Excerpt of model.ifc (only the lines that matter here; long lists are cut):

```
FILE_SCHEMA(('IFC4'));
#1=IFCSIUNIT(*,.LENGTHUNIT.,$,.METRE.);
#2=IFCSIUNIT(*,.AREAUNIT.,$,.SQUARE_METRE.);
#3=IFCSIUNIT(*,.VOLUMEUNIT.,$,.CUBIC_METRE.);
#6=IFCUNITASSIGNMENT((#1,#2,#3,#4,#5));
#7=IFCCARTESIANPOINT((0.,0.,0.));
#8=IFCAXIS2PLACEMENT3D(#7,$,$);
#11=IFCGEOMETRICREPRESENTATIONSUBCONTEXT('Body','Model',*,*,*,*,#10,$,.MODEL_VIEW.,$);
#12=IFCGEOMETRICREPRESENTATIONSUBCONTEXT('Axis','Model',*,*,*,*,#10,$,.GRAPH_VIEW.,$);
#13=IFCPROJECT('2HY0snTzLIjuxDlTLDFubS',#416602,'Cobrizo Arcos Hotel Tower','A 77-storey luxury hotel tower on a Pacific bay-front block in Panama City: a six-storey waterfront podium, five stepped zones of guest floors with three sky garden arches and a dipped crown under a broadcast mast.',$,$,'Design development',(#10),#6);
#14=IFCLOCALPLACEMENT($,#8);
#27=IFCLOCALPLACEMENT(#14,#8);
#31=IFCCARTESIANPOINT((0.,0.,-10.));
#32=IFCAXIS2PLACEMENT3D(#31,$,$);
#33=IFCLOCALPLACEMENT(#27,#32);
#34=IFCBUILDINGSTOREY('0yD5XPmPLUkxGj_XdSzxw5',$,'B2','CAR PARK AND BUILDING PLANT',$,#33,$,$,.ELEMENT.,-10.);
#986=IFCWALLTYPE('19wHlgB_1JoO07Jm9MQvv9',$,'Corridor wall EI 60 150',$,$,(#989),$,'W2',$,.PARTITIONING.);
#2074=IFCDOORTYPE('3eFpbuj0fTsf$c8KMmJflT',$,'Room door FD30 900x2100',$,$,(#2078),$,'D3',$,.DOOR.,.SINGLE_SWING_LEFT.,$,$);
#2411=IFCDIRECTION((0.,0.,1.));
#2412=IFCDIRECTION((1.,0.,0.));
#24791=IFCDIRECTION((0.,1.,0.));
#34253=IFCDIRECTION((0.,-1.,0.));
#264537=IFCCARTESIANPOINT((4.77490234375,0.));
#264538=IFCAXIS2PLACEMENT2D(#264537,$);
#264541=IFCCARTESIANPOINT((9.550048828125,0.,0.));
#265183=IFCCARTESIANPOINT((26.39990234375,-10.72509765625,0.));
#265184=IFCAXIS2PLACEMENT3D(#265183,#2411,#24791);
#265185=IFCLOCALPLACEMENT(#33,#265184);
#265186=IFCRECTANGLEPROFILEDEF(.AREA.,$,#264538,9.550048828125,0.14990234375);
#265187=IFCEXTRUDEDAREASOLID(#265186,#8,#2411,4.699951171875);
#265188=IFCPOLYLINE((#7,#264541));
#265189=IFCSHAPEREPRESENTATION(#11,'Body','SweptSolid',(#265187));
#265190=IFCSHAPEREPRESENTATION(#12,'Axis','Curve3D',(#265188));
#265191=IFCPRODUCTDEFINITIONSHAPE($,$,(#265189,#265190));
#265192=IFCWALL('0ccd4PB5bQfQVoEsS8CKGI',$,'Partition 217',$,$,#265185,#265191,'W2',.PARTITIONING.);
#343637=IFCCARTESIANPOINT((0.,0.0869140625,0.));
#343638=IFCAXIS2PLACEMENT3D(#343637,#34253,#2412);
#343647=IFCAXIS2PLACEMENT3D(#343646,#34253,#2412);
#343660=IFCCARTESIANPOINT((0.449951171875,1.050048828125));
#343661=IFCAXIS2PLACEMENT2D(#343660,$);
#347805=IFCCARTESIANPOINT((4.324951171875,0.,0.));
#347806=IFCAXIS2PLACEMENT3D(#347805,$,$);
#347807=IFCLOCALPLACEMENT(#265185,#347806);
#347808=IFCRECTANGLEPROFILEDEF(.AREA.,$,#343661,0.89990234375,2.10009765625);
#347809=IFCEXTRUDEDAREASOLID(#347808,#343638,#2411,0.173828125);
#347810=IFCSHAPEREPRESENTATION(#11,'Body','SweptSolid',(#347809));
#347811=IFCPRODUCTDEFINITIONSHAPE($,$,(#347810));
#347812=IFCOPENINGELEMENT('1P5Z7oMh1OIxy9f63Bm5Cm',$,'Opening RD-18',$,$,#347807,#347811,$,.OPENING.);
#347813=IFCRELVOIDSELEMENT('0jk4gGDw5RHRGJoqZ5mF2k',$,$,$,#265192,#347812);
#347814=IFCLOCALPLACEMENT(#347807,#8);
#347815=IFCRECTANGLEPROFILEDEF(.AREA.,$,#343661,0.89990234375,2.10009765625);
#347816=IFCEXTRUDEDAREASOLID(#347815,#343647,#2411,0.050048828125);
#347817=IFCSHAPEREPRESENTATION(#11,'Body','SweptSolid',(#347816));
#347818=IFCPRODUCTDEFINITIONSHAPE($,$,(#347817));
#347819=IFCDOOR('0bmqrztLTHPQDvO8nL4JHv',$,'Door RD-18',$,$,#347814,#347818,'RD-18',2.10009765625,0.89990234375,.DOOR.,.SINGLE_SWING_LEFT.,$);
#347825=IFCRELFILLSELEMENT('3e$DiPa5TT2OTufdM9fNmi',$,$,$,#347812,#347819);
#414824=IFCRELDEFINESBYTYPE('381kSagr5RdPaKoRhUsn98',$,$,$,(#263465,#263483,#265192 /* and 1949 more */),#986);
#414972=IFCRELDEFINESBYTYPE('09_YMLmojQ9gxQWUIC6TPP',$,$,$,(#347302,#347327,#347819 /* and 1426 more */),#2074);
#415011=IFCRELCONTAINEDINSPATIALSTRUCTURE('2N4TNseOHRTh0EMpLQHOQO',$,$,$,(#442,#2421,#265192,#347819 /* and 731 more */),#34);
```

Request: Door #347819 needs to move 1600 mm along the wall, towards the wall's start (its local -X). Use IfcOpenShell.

```python
import ifcopenshell
import ifcopenshell.api.geometry
import ifcopenshell.util.placement

model = ifcopenshell.open("model.ifc")

door = model.by_guid("0bmqrztLTHPQDvO8nL4JHv")
opening = door.FillsVoids[0].RelatingOpeningElement
wall = opening.VoidsElements[0].RelatingBuildingElement

wall_matrix = ifcopenshell.util.placement.get_local_placement(wall.ObjectPlacement)
shift = wall_matrix[:3, 0] * -1.6
before = ifcopenshell.util.placement.get_local_placement(door.ObjectPlacement)[:3, 3].copy()

# The door is placed relative to its opening, so it follows when the opening moves.
matrix = ifcopenshell.util.placement.get_local_placement(opening.ObjectPlacement)
matrix[:3, 3] += shift
ifcopenshell.api.geometry.edit_object_placement(
    model, product=opening, matrix=matrix, is_si=False, should_transform_children=True
)

after = ifcopenshell.util.placement.get_local_placement(door.ObjectPlacement)[:3, 3]
print("door moved by", (after - before).round(3) + 0.0)

model.write("model_rev.ifc")
```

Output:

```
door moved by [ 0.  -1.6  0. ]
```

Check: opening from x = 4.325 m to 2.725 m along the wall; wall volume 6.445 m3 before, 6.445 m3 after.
